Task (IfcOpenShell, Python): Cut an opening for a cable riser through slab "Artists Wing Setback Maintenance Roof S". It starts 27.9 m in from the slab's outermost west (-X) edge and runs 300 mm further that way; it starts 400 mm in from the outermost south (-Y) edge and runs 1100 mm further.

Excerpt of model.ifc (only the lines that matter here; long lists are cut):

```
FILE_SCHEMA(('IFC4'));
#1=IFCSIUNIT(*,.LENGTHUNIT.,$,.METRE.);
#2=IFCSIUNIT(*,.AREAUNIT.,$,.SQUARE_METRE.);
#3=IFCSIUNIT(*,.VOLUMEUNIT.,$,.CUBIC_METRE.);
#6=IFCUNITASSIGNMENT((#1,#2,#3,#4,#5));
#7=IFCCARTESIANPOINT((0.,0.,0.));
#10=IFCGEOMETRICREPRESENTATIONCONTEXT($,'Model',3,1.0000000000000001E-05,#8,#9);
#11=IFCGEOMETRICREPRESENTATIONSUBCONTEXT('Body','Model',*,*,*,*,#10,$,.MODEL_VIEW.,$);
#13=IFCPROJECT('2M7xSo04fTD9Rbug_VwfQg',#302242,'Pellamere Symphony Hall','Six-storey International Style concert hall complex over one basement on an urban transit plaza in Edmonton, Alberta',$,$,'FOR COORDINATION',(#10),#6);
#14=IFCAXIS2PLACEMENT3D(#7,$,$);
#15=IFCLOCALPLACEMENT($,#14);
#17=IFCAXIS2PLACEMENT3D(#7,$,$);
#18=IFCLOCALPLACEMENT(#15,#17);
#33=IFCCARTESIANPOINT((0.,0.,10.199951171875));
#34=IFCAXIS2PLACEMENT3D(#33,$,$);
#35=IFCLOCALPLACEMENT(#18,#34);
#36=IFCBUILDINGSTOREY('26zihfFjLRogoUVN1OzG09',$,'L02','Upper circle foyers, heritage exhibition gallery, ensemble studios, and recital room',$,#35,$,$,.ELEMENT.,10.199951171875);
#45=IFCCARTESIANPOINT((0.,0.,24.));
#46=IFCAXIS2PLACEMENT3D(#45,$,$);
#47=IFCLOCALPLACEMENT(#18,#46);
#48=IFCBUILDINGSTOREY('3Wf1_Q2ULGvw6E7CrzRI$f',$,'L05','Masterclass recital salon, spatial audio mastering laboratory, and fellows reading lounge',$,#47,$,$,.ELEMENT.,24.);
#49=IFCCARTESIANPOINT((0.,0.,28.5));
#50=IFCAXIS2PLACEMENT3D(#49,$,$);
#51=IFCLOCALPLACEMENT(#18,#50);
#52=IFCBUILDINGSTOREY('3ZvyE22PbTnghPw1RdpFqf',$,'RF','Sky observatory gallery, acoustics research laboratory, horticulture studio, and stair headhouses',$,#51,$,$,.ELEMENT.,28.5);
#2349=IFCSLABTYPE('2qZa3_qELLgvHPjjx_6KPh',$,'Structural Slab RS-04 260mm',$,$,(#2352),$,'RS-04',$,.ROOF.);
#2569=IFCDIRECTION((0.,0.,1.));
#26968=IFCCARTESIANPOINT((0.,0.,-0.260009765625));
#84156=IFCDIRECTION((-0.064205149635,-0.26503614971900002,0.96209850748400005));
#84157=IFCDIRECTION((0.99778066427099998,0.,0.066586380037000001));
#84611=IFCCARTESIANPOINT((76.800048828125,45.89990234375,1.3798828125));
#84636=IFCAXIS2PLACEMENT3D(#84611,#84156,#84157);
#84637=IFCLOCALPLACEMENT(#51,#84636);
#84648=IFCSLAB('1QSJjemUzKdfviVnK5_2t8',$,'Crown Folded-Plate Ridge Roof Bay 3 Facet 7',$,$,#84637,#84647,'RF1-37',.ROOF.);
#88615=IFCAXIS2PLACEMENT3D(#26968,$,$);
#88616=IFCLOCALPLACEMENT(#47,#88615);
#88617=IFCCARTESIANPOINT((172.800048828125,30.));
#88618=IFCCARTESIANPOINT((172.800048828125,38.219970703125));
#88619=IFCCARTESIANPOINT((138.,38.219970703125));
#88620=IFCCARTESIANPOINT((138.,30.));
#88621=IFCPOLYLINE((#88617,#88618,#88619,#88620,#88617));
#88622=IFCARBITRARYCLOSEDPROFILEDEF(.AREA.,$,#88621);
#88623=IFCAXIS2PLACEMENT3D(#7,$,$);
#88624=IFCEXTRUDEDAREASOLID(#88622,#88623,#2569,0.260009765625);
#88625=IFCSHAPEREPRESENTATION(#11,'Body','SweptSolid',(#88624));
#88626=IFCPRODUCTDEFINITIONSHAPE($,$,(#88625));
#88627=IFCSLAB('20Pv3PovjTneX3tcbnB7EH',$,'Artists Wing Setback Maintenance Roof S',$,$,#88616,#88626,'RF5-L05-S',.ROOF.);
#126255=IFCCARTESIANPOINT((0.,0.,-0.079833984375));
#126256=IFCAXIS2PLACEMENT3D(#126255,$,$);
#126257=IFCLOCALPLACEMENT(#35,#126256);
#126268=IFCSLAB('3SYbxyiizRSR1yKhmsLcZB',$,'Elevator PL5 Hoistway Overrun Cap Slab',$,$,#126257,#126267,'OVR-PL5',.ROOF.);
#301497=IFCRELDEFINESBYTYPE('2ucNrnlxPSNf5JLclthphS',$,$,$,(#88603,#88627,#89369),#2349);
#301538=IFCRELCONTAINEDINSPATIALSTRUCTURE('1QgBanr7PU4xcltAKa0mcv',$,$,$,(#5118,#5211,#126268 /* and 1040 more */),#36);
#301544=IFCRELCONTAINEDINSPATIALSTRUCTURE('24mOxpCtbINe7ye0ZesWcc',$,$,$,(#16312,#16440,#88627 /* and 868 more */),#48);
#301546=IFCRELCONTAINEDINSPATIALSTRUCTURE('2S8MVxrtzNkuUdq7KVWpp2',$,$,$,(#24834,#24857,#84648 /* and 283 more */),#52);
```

```python
import numpy as np
import ifcopenshell
import ifcopenshell.api.feature
import ifcopenshell.api.geometry
import ifcopenshell.api.root
import ifcopenshell.geom
import ifcopenshell.util.placement
import ifcopenshell.util.representation
import ifcopenshell.util.shape
import ifcopenshell.util.unit

model = ifcopenshell.open("model.ifc")
unit_scale = ifcopenshell.util.unit.calculate_unit_scale(model)
settings = ifcopenshell.geom.settings()


def volume(element):
    """Net volume in cubic metres, openings subtracted."""
    shape = ifcopenshell.geom.create_shape(settings, element)
    return ifcopenshell.util.shape.get_volume(shape.geometry)


slab = model.by_guid("20Pv3PovjTneX3tcbnB7EH")
before = volume(slab)

# Extent in the slab's own axes, in metres. The edges named are its -X and -Y sides.
slab_shape = ifcopenshell.geom.create_shape(settings, slab)
vertices = ifcopenshell.util.shape.get_vertices(slab_shape.geometry)
x_min, y_min, bottom = vertices.min(axis=0)
top = vertices[:, 2].max()

opening = ifcopenshell.api.root.create_entity(model, ifc_class="IfcOpeningElement", name="Cable riser opening", predefined_type="OPENING")
context = ifcopenshell.util.representation.get_context(model, "Model", "Body", "MODEL_VIEW")
width, depth = 0.3, 1.1
outline = [(0.0, 0.0), (width, 0.0), (width, depth), (0.0, depth), (0.0, 0.0)]
# Overshoot both faces by 50 mm so the cut is clean.
shape = ifcopenshell.api.geometry.add_slab_representation(
    model, context=context, depth=top - bottom + 0.1, polyline=outline
)
ifcopenshell.api.geometry.assign_representation(model, product=opening, representation=shape)

matrix = ifcopenshell.util.placement.get_local_placement(slab.ObjectPlacement)
matrix[:, 3] = matrix @ np.append(np.array([x_min + 27.9, y_min + 0.4, bottom - 0.05]) / unit_scale, 1.0)
ifcopenshell.api.geometry.edit_object_placement(model, product=opening, matrix=matrix, is_si=False)
ifcopenshell.api.feature.add_feature(model, feature=opening, element=slab)

after = volume(slab)

print(f"slab volume {before:.3f} -> {after:.3f} m3")

model.write("model_rev.ifc")
```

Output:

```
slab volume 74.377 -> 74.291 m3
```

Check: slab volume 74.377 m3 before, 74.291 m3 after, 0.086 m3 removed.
